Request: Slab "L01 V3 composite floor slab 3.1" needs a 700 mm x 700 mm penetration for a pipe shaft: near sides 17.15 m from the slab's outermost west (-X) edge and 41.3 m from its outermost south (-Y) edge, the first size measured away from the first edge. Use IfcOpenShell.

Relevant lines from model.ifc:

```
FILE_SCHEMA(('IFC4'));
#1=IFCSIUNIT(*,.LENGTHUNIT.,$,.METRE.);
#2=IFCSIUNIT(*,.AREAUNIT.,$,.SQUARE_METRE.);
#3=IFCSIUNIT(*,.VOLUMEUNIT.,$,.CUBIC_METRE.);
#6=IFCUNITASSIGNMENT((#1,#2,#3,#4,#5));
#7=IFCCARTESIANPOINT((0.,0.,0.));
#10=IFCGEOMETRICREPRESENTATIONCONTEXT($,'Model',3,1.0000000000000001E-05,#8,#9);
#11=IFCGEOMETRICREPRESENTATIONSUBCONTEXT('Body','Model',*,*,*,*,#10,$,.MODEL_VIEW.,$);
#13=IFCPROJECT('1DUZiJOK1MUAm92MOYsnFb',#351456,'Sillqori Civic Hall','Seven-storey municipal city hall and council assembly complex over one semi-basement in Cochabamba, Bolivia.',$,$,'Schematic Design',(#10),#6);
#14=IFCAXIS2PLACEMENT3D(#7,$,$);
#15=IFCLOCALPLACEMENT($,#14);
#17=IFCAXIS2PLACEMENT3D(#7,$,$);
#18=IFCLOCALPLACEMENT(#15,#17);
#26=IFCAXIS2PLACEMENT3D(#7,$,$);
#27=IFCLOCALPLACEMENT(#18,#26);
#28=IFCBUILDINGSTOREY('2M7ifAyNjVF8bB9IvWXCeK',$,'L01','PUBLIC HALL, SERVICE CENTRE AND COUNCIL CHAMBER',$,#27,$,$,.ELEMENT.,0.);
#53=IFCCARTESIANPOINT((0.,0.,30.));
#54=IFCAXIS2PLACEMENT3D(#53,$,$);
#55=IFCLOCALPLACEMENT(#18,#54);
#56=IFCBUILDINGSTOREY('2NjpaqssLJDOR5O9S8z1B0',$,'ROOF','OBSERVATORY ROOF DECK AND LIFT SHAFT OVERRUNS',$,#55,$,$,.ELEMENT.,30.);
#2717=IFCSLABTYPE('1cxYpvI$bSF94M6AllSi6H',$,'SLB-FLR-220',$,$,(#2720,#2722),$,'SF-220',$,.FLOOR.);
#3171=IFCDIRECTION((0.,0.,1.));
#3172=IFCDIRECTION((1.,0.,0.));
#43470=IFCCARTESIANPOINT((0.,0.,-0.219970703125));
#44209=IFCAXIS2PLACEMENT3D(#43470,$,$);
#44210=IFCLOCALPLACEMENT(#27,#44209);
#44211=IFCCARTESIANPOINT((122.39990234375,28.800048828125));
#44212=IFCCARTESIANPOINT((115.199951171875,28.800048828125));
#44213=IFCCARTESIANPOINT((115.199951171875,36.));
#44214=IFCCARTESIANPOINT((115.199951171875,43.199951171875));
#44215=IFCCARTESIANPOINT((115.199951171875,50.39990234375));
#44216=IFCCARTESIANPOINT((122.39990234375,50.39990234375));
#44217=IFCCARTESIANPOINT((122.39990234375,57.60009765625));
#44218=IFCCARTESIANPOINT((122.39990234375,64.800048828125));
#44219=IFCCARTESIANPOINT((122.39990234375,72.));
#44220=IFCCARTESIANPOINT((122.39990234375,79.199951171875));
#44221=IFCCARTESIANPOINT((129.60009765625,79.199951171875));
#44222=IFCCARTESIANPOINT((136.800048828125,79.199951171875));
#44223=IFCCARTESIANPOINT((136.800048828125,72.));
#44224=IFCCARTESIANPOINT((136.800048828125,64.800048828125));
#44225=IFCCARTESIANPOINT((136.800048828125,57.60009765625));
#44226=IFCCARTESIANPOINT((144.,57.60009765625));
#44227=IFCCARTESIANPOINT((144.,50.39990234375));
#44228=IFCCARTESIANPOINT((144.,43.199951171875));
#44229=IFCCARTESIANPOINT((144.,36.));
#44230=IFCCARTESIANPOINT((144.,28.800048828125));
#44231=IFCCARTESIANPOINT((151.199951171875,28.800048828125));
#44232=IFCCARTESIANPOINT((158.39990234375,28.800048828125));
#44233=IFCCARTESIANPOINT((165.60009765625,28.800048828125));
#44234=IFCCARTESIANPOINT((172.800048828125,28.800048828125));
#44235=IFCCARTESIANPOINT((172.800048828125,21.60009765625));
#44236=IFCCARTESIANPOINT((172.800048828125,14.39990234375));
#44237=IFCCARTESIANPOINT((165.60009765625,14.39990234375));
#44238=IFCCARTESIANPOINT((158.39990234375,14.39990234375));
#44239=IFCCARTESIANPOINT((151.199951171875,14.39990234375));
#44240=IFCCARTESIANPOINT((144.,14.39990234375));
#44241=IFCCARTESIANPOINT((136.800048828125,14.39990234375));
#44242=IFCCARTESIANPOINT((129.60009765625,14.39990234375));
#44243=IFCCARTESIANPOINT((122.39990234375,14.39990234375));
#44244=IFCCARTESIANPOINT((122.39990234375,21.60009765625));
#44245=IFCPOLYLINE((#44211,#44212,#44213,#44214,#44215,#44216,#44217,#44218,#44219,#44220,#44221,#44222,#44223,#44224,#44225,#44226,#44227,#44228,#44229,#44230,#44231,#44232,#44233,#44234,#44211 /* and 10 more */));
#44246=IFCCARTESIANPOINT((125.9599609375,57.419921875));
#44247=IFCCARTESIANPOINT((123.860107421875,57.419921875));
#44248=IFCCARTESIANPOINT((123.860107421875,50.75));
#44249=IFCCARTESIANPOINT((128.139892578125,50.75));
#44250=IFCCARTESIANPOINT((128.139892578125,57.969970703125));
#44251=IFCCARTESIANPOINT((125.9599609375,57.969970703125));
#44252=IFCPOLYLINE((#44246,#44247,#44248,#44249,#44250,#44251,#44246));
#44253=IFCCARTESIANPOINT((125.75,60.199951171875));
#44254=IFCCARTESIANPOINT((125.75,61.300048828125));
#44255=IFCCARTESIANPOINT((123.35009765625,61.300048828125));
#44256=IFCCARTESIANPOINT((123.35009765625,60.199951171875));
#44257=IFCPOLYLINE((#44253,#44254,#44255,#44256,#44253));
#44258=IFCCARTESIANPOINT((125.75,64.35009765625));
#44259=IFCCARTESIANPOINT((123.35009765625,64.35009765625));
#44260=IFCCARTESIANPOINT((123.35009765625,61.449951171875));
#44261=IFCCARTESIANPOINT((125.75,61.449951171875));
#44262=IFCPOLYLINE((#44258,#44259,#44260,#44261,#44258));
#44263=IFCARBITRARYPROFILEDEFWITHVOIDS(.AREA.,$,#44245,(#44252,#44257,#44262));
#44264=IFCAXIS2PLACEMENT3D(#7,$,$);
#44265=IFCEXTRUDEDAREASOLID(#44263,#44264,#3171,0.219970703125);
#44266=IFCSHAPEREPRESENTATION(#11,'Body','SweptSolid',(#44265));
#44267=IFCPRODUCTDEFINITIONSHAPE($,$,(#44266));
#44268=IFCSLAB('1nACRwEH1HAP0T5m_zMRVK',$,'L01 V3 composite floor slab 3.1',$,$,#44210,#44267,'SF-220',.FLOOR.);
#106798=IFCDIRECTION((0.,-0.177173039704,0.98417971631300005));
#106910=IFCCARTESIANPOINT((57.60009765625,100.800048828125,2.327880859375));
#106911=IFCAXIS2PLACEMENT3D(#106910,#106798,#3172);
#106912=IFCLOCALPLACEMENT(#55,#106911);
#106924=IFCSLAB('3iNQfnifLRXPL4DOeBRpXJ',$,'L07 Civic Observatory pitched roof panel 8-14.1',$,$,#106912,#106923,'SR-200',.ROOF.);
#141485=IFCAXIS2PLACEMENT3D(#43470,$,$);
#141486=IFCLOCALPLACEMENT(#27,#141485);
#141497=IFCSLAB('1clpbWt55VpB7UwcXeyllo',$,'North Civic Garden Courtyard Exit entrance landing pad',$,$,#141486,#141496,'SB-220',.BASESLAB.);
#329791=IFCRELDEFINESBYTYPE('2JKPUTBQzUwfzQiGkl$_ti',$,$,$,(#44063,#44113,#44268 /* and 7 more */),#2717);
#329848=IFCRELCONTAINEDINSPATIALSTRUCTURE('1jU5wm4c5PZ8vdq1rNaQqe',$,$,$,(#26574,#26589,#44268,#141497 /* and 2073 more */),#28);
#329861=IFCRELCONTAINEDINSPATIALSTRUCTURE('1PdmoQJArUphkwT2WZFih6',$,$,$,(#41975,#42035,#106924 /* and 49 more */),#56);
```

```python
import numpy as np
import ifcopenshell
import ifcopenshell.api.feature
import ifcopenshell.api.geometry
import ifcopenshell.api.root
import ifcopenshell.geom
import ifcopenshell.util.placement
import ifcopenshell.util.representation
import ifcopenshell.util.shape
import ifcopenshell.util.unit

model = ifcopenshell.open("model.ifc")
unit_scale = ifcopenshell.util.unit.calculate_unit_scale(model)
settings = ifcopenshell.geom.settings()


def volume(element):
    """Net volume in cubic metres, openings subtracted."""
    shape = ifcopenshell.geom.create_shape(settings, element)
    return ifcopenshell.util.shape.get_volume(shape.geometry)


slab = model.by_id(44268)
before = volume(slab)

# Extent in the slab's own axes, in metres. The edges named are its -X and -Y sides.
slab_shape = ifcopenshell.geom.create_shape(settings, slab)
vertices = ifcopenshell.util.shape.get_vertices(slab_shape.geometry)
x_min, y_min, bottom = vertices.min(axis=0)
top = vertices[:, 2].max()

opening = ifcopenshell.api.root.create_entity(model, ifc_class="IfcOpeningElement", name="Pipe shaft opening", predefined_type="OPENING")
context = ifcopenshell.util.representation.get_context(model, "Model", "Body", "MODEL_VIEW")
width, depth = 0.7, 0.7
outline = [(0.0, 0.0), (width, 0.0), (width, depth), (0.0, depth), (0.0, 0.0)]
# Overshoot both faces by 50 mm so the cut is clean.
shape = ifcopenshell.api.geometry.add_slab_representation(
    model, context=context, depth=top - bottom + 0.1, polyline=outline
)
ifcopenshell.api.geometry.assign_representation(model, product=opening, representation=shape)

matrix = ifcopenshell.util.placement.get_local_placement(slab.ObjectPlacement)
matrix[:, 3] = matrix @ np.append(np.array([x_min + 17.15, y_min + 41.3, bottom - 0.05]) / unit_scale, 1.0)
ifcopenshell.api.geometry.edit_object_placement(model, product=opening, matrix=matrix, is_si=False)
ifcopenshell.api.feature.add_feature(model, feature=opening, element=slab)

after = volume(slab)

print(f"slab volume {before:.3f} -> {after:.3f} m3")

model.write("model-out.ifc")
```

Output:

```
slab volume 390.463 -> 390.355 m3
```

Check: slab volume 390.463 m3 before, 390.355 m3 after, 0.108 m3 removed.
